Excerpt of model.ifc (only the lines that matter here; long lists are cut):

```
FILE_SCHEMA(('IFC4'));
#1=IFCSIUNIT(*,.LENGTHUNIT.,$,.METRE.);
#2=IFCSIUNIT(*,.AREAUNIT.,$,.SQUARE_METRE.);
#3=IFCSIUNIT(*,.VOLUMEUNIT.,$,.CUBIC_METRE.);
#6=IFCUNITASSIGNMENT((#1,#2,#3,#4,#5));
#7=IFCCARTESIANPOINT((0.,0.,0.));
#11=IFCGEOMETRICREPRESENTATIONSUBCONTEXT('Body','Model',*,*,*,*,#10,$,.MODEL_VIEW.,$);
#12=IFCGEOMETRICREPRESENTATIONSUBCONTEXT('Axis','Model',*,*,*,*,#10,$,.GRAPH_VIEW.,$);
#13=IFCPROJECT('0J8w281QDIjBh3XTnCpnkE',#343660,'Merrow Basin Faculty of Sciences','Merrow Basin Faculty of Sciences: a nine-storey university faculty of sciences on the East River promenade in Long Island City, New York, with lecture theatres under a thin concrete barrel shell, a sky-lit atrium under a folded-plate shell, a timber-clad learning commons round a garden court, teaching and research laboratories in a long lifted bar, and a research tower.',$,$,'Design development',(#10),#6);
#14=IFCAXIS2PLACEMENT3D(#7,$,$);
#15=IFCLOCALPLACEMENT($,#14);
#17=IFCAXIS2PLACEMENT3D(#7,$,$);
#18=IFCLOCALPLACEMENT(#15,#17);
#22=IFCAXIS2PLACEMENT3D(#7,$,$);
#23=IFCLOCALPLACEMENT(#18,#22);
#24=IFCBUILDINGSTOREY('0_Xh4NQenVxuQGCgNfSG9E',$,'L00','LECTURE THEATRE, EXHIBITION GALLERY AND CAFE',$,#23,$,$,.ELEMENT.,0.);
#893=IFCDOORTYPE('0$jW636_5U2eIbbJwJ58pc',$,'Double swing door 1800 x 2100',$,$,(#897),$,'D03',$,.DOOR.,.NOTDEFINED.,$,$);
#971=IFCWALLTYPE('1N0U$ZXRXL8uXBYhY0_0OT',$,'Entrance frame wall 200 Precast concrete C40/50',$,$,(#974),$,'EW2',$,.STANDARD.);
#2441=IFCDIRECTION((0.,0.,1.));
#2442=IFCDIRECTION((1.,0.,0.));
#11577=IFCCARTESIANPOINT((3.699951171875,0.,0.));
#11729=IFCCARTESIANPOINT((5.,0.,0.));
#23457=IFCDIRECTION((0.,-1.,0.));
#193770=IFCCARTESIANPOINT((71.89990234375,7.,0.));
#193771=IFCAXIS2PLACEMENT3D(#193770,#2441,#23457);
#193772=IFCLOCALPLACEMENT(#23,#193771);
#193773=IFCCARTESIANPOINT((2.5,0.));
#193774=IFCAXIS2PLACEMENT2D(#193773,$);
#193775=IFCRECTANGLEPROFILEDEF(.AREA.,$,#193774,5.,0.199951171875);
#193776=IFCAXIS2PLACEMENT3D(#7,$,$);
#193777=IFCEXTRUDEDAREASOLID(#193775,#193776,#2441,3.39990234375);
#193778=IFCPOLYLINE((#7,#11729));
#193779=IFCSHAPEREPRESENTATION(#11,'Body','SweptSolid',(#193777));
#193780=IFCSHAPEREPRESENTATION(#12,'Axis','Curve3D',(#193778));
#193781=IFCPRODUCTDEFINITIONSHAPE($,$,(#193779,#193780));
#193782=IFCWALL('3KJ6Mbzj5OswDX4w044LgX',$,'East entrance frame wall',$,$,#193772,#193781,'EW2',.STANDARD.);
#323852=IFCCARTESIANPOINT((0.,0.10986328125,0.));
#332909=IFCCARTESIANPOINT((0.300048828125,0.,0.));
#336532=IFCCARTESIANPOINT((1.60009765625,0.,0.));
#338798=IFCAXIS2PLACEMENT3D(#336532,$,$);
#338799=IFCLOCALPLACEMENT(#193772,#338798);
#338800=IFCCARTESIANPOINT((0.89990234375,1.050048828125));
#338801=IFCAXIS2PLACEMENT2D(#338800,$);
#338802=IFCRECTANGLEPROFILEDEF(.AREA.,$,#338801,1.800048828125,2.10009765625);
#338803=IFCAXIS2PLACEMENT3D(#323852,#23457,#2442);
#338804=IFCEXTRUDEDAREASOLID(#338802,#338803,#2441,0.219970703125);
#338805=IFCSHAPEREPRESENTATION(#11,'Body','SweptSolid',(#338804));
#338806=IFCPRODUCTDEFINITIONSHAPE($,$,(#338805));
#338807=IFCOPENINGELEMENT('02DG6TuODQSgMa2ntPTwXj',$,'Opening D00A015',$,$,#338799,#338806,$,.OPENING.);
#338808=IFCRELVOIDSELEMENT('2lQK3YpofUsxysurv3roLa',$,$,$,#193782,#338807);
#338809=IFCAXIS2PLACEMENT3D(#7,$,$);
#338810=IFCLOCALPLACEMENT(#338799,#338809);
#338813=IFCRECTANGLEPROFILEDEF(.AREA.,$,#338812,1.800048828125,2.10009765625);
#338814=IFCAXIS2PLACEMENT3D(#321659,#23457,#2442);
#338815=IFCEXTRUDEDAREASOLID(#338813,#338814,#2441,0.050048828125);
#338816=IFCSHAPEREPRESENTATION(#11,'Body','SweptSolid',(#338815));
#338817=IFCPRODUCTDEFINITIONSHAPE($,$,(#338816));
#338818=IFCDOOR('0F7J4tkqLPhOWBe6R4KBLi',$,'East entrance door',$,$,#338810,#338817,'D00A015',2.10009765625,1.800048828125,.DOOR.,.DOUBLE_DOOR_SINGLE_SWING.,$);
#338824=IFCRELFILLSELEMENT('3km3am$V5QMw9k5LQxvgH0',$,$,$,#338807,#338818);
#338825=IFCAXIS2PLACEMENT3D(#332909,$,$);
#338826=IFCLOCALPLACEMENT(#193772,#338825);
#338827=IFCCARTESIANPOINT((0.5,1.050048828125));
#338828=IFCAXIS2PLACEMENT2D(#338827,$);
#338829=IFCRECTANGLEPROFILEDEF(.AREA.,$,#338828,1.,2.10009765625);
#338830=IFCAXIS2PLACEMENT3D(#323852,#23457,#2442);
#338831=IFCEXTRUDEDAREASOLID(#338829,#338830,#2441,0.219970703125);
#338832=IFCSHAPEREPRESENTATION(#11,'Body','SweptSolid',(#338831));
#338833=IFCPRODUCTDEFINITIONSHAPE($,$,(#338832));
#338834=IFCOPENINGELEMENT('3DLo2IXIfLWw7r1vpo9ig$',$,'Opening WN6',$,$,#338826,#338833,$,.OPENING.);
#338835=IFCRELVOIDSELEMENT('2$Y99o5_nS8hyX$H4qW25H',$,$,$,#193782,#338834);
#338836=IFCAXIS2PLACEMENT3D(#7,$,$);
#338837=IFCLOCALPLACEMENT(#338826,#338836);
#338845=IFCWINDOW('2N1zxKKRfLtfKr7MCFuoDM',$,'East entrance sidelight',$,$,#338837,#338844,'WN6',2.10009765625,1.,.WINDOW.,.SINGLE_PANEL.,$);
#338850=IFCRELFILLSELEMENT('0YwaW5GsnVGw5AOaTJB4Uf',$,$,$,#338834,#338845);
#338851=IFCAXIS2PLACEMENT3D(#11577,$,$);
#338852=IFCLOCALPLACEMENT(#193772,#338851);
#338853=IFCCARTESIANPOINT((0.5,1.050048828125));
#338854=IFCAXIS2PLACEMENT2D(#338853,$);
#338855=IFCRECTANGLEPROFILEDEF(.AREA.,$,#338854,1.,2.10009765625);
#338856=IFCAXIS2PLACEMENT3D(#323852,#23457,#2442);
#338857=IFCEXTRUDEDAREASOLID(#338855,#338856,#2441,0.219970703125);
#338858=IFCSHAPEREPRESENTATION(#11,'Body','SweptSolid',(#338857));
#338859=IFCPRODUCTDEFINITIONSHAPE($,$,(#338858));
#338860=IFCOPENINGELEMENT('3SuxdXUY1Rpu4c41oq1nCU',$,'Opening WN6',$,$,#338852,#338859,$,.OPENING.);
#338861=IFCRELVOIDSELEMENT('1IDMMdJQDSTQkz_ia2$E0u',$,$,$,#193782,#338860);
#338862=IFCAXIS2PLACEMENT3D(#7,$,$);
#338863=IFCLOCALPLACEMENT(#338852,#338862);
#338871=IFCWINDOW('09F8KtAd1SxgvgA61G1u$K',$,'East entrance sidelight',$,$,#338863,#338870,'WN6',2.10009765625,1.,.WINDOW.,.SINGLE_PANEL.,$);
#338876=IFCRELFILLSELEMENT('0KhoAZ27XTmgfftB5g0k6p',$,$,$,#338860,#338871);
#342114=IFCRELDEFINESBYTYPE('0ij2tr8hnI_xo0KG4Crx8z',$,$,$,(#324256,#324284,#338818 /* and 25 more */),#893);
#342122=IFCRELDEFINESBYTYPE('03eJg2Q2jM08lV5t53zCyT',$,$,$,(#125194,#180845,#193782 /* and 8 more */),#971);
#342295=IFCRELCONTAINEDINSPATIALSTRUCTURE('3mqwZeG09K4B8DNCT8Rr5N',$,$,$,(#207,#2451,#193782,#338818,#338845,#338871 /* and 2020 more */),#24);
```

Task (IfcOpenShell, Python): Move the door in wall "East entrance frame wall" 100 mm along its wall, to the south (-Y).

```python
import ifcopenshell
import ifcopenshell.api.geometry
import ifcopenshell.util.placement
import ifcopenshell.util.unit

model = ifcopenshell.open("model.ifc")
unit_scale = ifcopenshell.util.unit.calculate_unit_scale(model)

door = model.by_id(338818)
opening = door.FillsVoids[0].RelatingOpeningElement
wall = opening.VoidsElements[0].RelatingBuildingElement

wall_matrix = ifcopenshell.util.placement.get_local_placement(wall.ObjectPlacement)
shift = wall_matrix[:3, 0] * 0.1 / unit_scale
before = ifcopenshell.util.placement.get_local_placement(door.ObjectPlacement)[:3, 3].copy()

# The door is placed relative to its opening, so it follows when the opening moves.
matrix = ifcopenshell.util.placement.get_local_placement(opening.ObjectPlacement)
matrix[:3, 3] += shift
ifcopenshell.api.geometry.edit_object_placement(
    model, product=opening, matrix=matrix, is_si=False, should_transform_children=True
)

after = ifcopenshell.util.placement.get_local_placement(door.ObjectPlacement)[:3, 3]
print("door moved by", (after - before).round(3) + 0.0)

model.write("model_v2.ifc")
```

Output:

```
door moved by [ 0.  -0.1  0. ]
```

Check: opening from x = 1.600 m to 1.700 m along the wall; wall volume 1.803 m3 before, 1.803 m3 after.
